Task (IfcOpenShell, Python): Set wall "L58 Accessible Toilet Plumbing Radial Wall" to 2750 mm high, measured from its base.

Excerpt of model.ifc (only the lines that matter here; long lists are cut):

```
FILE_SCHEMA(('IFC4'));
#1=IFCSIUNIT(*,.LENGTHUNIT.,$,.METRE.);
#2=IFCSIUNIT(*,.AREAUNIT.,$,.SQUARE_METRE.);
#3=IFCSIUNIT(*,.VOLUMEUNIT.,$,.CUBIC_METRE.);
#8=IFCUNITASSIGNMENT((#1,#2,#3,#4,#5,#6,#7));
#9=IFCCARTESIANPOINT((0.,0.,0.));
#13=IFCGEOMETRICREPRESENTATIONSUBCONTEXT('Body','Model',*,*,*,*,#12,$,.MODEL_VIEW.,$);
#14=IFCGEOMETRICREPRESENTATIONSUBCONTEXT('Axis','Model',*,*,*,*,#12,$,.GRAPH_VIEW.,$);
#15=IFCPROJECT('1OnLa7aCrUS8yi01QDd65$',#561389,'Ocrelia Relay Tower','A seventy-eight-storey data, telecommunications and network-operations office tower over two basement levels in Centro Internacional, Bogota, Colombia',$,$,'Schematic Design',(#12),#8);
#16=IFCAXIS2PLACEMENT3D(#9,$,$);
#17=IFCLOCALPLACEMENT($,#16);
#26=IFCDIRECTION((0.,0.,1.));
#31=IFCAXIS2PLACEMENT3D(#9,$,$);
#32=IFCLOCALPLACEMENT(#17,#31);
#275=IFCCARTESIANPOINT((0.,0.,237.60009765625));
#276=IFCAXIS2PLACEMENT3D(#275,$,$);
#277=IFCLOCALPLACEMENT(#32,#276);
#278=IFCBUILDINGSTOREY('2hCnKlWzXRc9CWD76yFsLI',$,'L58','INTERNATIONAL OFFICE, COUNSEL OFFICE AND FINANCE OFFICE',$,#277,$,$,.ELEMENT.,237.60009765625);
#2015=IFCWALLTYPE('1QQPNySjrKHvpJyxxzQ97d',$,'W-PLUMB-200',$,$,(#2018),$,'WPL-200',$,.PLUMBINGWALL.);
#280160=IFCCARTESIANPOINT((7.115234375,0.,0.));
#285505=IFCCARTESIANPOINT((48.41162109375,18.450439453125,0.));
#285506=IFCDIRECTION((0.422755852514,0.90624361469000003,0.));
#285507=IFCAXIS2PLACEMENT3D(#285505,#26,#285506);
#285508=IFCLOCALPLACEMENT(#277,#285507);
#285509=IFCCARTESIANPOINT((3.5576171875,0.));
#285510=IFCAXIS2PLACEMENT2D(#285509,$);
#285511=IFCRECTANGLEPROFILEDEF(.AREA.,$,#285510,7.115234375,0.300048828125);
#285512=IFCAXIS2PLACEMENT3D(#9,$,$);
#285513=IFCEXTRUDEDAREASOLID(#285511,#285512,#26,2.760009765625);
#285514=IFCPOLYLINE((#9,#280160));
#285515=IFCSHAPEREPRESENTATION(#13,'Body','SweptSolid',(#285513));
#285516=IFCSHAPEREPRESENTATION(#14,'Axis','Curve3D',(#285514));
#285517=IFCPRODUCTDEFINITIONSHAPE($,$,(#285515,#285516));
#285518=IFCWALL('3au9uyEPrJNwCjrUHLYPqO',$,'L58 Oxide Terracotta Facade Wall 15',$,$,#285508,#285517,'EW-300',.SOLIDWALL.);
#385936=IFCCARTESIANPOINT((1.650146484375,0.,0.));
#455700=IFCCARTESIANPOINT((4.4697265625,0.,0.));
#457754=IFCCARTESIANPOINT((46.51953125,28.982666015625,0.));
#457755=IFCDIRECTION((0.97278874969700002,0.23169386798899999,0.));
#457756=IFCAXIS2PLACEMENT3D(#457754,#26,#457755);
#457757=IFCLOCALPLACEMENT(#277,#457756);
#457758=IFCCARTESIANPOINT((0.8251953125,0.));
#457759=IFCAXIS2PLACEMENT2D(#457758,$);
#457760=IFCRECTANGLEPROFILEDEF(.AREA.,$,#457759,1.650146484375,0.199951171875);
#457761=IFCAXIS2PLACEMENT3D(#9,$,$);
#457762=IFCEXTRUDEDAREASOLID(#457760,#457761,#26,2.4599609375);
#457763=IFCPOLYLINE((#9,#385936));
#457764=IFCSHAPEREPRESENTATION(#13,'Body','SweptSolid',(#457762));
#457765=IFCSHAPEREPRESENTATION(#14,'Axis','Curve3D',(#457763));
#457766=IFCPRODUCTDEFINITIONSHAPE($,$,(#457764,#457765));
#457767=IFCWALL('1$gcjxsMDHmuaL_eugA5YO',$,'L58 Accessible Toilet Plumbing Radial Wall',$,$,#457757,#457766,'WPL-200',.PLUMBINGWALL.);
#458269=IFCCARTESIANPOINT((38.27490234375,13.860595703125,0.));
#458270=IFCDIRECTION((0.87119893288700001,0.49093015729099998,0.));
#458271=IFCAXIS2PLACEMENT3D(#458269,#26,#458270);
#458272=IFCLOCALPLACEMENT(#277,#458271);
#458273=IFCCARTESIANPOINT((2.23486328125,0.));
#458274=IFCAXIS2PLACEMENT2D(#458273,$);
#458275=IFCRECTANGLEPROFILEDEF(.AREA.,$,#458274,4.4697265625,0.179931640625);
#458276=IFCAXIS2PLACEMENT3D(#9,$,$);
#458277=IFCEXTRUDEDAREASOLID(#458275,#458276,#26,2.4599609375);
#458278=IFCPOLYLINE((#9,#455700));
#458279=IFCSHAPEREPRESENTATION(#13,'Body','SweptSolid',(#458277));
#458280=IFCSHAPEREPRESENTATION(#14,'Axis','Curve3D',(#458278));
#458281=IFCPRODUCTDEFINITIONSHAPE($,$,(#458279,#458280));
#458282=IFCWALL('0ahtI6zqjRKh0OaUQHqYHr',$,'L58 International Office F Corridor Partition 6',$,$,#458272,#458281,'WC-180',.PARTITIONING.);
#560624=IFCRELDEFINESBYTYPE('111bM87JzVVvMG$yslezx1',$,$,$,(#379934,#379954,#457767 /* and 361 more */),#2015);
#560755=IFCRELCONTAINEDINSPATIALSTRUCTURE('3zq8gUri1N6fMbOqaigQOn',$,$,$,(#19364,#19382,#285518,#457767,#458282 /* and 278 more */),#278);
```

```python
import ifcopenshell
import ifcopenshell.geom
import ifcopenshell.util.representation
import ifcopenshell.util.shape

model = ifcopenshell.open("model.ifc")
settings = ifcopenshell.geom.settings()


def volume(element):
    """Net volume in cubic metres, openings subtracted."""
    shape = ifcopenshell.geom.create_shape(settings, element)
    return ifcopenshell.util.shape.get_volume(shape.geometry)


wall = model.by_id(457767)
before = volume(wall)

body = ifcopenshell.util.representation.get_representation(wall, "Model", "Body")
solid = body.Items[0]
old_height = solid.Depth
solid.Depth = 2.75
after = volume(wall)

print(f"height {old_height:g} -> {solid.Depth:g}, volume {before:.3f} -> {after:.3f} m3")

model.write("model_rev.ifc")
```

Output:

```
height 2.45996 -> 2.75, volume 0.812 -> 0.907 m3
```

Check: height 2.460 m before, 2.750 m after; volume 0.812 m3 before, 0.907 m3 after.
